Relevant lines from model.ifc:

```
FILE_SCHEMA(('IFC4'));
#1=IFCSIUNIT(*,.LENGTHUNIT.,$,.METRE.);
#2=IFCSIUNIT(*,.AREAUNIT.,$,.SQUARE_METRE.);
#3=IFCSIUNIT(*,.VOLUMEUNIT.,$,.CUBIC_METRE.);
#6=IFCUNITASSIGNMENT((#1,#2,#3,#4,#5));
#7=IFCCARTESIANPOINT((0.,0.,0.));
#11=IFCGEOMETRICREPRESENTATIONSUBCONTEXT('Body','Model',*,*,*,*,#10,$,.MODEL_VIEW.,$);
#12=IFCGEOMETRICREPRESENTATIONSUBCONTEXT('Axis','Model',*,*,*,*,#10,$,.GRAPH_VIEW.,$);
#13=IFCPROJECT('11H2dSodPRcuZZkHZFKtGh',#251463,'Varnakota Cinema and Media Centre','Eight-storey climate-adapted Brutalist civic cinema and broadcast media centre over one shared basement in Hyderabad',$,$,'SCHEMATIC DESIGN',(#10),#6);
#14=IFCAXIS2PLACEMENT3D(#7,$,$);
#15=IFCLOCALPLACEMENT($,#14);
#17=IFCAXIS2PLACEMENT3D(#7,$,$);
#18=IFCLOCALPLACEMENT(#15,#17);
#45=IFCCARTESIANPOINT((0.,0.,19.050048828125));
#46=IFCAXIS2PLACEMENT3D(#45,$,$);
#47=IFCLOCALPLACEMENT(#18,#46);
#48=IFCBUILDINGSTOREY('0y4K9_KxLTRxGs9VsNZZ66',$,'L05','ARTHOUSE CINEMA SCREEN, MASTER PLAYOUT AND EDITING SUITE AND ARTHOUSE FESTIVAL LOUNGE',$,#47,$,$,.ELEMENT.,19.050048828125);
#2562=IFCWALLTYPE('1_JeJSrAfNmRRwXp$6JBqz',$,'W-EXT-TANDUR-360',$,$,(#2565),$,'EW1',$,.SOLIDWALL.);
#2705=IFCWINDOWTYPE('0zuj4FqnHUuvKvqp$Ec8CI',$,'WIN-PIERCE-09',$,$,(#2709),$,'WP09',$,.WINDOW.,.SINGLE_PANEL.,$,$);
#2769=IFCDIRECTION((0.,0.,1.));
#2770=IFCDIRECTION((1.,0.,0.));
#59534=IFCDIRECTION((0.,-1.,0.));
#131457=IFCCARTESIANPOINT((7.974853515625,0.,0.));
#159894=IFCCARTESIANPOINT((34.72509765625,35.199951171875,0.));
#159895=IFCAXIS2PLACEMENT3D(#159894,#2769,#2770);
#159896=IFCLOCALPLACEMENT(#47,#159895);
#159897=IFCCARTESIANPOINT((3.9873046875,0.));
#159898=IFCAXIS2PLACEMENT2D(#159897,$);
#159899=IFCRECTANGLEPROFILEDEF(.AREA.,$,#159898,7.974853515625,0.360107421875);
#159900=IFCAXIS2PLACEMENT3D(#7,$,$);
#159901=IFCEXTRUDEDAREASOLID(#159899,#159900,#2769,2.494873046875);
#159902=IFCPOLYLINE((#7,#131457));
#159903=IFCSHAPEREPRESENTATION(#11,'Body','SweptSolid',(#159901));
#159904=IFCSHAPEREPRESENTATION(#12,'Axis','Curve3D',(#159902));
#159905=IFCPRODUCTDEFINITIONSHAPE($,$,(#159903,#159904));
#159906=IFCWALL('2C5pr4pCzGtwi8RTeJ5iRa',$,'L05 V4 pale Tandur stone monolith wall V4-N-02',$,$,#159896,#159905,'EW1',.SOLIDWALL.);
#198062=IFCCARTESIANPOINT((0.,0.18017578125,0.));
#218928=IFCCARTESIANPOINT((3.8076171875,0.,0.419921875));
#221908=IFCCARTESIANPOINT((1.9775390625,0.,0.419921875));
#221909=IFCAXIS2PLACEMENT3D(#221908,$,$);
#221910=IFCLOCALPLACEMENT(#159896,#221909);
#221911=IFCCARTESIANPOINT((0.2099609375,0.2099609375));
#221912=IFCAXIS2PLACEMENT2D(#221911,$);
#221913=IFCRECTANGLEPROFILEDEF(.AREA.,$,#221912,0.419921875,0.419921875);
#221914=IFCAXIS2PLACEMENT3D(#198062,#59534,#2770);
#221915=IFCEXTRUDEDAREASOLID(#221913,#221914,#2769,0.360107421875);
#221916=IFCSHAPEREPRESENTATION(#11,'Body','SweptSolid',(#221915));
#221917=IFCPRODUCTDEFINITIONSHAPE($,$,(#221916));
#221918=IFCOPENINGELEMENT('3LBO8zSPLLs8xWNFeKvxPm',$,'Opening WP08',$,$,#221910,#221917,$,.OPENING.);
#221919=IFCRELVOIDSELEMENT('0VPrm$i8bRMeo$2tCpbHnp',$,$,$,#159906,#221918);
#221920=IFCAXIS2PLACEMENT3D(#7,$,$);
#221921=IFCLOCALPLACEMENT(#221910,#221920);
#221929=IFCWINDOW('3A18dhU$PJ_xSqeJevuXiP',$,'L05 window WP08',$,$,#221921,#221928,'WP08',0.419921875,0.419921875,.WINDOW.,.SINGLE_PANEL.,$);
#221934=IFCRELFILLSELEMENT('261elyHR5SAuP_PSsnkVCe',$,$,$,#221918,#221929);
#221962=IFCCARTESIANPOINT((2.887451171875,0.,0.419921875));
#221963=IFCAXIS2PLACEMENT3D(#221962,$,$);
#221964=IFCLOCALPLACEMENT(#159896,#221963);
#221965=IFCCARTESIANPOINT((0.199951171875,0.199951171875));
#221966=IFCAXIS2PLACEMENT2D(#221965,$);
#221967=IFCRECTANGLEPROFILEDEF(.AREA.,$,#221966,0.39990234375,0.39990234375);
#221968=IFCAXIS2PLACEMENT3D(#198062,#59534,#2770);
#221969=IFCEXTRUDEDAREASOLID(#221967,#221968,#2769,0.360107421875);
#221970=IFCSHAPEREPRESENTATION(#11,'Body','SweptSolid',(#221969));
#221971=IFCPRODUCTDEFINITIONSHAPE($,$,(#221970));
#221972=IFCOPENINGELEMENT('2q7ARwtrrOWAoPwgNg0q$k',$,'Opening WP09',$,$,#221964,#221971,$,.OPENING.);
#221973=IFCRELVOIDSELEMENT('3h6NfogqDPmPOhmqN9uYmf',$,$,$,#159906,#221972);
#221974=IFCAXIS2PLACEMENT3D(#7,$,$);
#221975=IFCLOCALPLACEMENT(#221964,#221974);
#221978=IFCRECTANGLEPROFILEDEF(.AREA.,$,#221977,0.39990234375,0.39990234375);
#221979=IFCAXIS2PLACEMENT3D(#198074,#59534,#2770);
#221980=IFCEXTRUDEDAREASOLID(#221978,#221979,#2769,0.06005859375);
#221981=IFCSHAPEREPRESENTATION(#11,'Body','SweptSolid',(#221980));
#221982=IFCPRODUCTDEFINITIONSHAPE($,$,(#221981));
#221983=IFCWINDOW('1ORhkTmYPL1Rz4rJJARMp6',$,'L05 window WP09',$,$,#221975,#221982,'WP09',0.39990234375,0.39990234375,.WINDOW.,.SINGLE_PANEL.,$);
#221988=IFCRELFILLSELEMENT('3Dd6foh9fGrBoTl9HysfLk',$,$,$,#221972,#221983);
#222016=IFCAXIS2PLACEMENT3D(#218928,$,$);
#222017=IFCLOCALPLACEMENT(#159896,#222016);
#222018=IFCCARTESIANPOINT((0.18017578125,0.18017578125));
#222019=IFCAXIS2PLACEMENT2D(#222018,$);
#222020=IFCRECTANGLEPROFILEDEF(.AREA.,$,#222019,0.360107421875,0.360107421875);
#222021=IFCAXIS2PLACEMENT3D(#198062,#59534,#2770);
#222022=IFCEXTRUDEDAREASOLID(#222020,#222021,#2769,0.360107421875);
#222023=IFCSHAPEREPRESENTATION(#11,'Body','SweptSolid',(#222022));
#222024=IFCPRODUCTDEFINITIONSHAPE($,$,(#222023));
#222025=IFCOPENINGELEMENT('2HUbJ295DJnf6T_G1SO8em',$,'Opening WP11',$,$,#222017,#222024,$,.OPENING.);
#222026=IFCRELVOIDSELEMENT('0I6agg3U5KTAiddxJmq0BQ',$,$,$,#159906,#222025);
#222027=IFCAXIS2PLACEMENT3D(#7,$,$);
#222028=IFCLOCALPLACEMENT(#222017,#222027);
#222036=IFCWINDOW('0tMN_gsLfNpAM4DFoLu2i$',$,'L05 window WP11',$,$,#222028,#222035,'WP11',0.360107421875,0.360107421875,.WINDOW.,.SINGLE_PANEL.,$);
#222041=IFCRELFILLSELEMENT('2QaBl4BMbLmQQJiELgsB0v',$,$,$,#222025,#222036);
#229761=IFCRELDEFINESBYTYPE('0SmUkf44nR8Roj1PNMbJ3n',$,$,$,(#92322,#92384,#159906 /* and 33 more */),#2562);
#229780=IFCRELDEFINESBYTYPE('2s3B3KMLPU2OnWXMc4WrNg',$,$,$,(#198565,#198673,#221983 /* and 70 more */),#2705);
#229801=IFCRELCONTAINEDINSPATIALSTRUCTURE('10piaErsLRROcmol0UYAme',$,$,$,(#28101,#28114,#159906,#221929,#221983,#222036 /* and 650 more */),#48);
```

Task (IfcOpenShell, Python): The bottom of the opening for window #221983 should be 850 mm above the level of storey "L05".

```python
import numpy as np
import ifcopenshell
import ifcopenshell.api.geometry
import ifcopenshell.geom
import ifcopenshell.util.element
import ifcopenshell.util.placement
import ifcopenshell.util.shape
import ifcopenshell.util.unit

model = ifcopenshell.open("model.ifc")
unit_scale = ifcopenshell.util.unit.calculate_unit_scale(model)

window = model.by_id(221983)
opening = window.FillsVoids[0].RelatingOpeningElement
storey = ifcopenshell.util.element.get_container(window, ifc_class="IfcBuildingStorey")
level = ifcopenshell.util.placement.get_local_placement(storey.ObjectPlacement)[2, 3]

# The opening's origin need not be at the sill, so measure its lowest point.
shape = ifcopenshell.geom.create_shape(ifcopenshell.geom.settings(), opening)
bottom = ifcopenshell.util.shape.get_shape_bottom_elevation(shape, shape.geometry) / unit_scale
dz = level + 0.85 / unit_scale - bottom

shift = np.array([0.0, 0.0, dz])
# The window is placed relative to its opening, so it follows when the opening moves.
matrix = ifcopenshell.util.placement.get_local_placement(opening.ObjectPlacement)
matrix[:3, 3] += shift
ifcopenshell.api.geometry.edit_object_placement(
    model, product=opening, matrix=matrix, is_si=False, should_transform_children=True
)

print(f"moved by {dz * unit_scale:+.3f} m")

model.write("model_edited.ifc")
```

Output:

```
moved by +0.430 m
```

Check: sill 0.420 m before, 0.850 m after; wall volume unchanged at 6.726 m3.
